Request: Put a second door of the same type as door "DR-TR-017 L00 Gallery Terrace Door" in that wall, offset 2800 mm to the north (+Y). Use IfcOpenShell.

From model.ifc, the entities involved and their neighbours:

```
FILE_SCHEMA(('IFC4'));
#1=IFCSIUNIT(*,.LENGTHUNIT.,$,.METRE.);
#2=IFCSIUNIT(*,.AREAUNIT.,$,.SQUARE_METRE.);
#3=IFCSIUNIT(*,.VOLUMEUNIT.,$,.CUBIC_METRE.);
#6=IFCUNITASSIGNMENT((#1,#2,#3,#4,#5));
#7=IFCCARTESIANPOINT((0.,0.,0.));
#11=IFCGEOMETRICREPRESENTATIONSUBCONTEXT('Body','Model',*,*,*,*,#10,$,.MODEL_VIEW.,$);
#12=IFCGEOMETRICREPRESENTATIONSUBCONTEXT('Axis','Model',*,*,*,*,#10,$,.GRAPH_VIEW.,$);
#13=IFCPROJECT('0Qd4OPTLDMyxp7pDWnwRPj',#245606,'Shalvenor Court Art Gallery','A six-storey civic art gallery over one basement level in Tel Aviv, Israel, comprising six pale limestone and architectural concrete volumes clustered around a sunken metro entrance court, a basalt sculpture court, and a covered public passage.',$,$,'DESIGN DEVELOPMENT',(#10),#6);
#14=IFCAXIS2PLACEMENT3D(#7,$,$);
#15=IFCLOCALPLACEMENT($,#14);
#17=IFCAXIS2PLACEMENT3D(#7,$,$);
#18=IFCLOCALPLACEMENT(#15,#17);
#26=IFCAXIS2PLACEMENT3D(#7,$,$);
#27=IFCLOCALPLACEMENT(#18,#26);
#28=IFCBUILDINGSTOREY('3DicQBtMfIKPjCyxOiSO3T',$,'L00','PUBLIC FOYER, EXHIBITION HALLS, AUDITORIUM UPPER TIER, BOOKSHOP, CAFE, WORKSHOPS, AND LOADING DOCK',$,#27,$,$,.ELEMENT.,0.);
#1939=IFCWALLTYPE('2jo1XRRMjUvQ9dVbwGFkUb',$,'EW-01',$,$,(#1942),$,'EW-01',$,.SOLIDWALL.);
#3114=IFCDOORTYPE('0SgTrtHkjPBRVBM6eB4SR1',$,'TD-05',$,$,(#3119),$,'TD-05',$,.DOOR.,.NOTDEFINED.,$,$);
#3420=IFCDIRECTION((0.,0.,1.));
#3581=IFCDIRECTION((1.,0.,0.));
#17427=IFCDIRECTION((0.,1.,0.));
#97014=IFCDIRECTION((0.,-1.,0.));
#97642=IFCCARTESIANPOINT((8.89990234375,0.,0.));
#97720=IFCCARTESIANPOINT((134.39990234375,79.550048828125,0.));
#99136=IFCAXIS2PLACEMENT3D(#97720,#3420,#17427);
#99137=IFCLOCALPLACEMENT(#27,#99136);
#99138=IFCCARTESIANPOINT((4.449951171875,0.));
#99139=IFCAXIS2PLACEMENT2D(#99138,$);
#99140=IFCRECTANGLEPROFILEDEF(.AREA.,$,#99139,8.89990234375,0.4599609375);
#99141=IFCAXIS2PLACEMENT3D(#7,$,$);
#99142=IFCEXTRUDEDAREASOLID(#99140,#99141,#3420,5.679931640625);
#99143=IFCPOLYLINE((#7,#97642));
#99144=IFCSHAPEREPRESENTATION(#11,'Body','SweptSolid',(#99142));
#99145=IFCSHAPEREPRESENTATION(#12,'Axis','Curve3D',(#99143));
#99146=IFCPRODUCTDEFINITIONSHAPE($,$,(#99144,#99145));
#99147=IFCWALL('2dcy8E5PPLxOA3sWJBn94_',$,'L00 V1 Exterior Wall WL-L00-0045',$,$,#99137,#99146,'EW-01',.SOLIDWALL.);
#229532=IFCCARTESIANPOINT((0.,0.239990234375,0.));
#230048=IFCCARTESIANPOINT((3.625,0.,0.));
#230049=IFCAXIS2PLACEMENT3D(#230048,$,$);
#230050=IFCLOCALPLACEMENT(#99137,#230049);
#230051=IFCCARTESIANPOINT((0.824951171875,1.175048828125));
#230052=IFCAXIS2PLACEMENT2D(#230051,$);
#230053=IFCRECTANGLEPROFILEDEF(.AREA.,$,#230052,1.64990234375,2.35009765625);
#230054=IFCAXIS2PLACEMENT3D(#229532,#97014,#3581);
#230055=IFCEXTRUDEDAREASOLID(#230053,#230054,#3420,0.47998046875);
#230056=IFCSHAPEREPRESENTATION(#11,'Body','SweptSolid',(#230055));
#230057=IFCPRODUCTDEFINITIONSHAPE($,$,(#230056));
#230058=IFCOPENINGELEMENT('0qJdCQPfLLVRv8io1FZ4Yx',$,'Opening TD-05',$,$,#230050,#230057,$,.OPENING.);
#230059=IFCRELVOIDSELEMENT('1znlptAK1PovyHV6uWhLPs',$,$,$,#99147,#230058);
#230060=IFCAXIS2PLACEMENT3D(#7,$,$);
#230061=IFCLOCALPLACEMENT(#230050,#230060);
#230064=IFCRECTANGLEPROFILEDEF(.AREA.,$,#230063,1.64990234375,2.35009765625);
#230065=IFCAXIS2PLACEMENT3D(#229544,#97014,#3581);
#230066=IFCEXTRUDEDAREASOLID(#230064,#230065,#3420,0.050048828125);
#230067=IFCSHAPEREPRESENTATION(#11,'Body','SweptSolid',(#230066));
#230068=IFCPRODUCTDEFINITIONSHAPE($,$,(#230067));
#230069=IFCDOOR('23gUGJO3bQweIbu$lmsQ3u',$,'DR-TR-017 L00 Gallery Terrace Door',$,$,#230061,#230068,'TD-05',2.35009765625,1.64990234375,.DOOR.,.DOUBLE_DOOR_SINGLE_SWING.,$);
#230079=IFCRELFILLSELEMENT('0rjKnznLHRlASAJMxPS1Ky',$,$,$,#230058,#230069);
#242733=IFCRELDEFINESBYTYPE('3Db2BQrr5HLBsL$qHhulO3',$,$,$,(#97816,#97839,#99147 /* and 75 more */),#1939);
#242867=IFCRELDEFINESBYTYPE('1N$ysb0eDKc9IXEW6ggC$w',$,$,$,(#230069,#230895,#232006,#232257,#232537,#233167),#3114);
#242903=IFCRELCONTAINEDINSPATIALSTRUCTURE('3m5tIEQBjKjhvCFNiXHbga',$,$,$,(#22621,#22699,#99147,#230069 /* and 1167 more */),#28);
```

```python
import ifcopenshell
import ifcopenshell.api.feature
import ifcopenshell.api.geometry
import ifcopenshell.api.root
import ifcopenshell.geom
import ifcopenshell.util.element
import ifcopenshell.util.placement
import ifcopenshell.util.shape

model = ifcopenshell.open("model.ifc")
settings = ifcopenshell.geom.settings()


def volume(element):
    """Net volume in cubic metres, openings subtracted."""
    shape = ifcopenshell.geom.create_shape(settings, element)
    return ifcopenshell.util.shape.get_volume(shape.geometry)


door = model.by_id(230069)
opening = door.FillsVoids[0].RelatingOpeningElement
wall = opening.VoidsElements[0].RelatingBuildingElement
before = volume(wall)
shift = ifcopenshell.util.placement.get_local_placement(wall.ObjectPlacement)[:3, 0] * 2.8

# copy_class copies the void relationship, type, container and properties, but no geometry.
new_opening = ifcopenshell.api.root.copy_class(model, product=opening)
new_opening.Representation = ifcopenshell.util.element.copy_deep(
    model, opening.Representation, exclude=["IfcGeometricRepresentationContext", "IfcRepresentationMap"]
)
new_door = ifcopenshell.api.root.copy_class(model, product=door)
new_door.Representation = ifcopenshell.util.element.copy_deep(
    model, door.Representation, exclude=["IfcGeometricRepresentationContext", "IfcRepresentationMap"]
)
new_door.Tag = None
ifcopenshell.api.feature.add_filling(model, opening=new_opening, element=new_door)

for old, new in ((opening, new_opening), (door, new_door)):
    matrix = ifcopenshell.util.placement.get_local_placement(old.ObjectPlacement)
    matrix[:3, 3] += shift
    ifcopenshell.api.geometry.edit_object_placement(model, product=new, matrix=matrix, is_si=False)

after = volume(wall)

print(f"wall volume {before:.3f} -> {after:.3f} m3")

model.write("model_v2.ifc")
```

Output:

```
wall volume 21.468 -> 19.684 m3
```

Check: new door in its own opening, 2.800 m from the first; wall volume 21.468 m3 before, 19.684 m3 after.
